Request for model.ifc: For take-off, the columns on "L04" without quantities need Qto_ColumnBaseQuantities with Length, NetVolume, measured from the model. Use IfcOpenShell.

First a look at what the model holds.

```python
import ifcopenshell
import ifcopenshell.util.element
import ifcopenshell.util.unit

model = ifcopenshell.open("model.ifc")
print(model.schema)
for unit_type in ("LENGTHUNIT", "AREAUNIT", "VOLUMEUNIT"):
    print(unit_type, ifcopenshell.util.unit.calculate_unit_scale(model, unit_type))
storey = next(s for s in model.by_type("IfcBuildingStorey") if s.Name == "L04")
columns = [e for e in ifcopenshell.util.element.get_decomposition(storey) if e.is_a("IfcColumn")]
for e in sorted(columns, key=lambda e: e.id()):
    print(e.id(), e.is_a(), e.Name, list(ifcopenshell.util.element.get_psets(e, qtos_only=True)), sep=" | ")
```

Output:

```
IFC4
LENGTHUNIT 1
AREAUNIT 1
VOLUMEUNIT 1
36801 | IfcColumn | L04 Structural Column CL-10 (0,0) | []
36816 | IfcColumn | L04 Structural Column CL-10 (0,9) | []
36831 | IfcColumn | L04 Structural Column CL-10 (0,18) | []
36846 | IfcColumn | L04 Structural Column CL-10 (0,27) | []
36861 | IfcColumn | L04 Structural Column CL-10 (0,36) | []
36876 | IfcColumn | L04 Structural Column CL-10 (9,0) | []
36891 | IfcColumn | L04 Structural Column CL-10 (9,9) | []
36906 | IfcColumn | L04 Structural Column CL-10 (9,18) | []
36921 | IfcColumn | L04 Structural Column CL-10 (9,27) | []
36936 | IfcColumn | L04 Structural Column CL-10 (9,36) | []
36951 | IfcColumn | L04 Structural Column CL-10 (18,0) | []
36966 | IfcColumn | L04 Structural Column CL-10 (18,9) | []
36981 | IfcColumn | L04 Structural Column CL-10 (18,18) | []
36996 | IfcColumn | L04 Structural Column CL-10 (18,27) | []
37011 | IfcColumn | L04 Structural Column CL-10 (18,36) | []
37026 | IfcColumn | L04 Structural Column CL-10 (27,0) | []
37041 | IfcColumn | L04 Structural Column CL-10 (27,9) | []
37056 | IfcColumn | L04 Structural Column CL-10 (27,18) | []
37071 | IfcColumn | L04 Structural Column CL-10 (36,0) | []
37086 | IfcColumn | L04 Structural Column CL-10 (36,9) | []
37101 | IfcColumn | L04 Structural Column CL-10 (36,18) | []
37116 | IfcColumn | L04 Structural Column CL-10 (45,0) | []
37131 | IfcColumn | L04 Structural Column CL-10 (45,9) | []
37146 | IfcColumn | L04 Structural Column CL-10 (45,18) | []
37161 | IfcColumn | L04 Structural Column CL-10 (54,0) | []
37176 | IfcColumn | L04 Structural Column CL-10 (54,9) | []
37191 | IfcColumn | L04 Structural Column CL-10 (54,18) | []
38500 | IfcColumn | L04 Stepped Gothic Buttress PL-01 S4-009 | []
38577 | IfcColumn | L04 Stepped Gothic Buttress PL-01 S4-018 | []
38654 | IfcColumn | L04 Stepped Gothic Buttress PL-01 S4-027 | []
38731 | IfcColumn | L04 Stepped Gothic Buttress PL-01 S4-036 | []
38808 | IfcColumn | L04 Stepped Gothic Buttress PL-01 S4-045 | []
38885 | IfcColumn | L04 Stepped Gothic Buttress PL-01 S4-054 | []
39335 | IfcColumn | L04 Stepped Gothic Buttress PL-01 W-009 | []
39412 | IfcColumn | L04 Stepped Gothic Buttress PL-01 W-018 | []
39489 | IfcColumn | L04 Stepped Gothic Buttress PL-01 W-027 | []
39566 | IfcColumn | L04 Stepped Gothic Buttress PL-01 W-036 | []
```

```python
import ifcopenshell
import ifcopenshell.api.pset
import ifcopenshell.geom
import ifcopenshell.util.element
import ifcopenshell.util.shape
import ifcopenshell.util.unit

model = ifcopenshell.open("model.ifc")
unit_scale = ifcopenshell.util.unit.calculate_unit_scale(model)
volume_scale = ifcopenshell.util.unit.calculate_unit_scale(model, "VOLUMEUNIT")
settings = ifcopenshell.geom.settings()

storey = next(s for s in model.by_type("IfcBuildingStorey") if s.Name == "L04")
columns = [e for e in ifcopenshell.util.element.get_decomposition(storey) if e.is_a("IfcColumn")]

for e in sorted(columns, key=lambda e: e.id()):
    if ifcopenshell.util.element.get_psets(e, qtos_only=True, should_inherit=False):
        continue
    # Geometry comes back in metres, in the element's own axes.
    shape = ifcopenshell.geom.create_shape(settings, e)
    values = {
        "Length": ifcopenshell.util.shape.get_z(shape.geometry) / unit_scale,
        "NetVolume": ifcopenshell.util.shape.get_volume(shape.geometry) / volume_scale,
    }
    qto = ifcopenshell.api.pset.add_qto(model, product=e, name="Qto_ColumnBaseQuantities")
    ifcopenshell.api.pset.edit_qto(model, qto=qto, properties=values)
    print(e.id(), {k: round(v, 3) for k, v in values.items()})

model.write("model_rev.ifc")
```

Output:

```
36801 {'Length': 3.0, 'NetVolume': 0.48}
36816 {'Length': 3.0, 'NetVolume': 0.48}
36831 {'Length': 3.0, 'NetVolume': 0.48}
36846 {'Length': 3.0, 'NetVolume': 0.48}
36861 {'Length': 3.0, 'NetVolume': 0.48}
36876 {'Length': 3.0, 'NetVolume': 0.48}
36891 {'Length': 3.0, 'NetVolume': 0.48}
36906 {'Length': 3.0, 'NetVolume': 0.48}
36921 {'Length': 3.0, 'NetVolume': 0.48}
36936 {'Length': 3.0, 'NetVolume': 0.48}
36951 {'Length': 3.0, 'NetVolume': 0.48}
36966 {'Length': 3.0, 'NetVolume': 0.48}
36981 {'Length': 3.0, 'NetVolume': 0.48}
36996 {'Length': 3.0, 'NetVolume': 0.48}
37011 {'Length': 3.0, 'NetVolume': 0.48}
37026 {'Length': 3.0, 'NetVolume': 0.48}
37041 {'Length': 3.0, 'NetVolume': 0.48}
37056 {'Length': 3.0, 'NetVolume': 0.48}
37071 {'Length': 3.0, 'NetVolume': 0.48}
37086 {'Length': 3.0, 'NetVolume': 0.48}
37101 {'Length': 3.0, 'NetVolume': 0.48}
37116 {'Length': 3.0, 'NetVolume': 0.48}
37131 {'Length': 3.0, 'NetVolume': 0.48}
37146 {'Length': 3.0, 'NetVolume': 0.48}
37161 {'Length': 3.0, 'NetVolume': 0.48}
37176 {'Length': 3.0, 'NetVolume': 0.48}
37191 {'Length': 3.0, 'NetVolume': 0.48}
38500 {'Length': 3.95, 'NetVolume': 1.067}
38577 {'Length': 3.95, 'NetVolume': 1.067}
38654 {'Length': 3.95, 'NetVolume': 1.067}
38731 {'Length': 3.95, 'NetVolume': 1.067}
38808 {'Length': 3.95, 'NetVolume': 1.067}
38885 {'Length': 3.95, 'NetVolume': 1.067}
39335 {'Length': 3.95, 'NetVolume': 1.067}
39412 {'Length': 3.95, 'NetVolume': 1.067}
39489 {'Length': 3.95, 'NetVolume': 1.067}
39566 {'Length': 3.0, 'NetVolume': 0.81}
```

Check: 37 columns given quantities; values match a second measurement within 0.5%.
